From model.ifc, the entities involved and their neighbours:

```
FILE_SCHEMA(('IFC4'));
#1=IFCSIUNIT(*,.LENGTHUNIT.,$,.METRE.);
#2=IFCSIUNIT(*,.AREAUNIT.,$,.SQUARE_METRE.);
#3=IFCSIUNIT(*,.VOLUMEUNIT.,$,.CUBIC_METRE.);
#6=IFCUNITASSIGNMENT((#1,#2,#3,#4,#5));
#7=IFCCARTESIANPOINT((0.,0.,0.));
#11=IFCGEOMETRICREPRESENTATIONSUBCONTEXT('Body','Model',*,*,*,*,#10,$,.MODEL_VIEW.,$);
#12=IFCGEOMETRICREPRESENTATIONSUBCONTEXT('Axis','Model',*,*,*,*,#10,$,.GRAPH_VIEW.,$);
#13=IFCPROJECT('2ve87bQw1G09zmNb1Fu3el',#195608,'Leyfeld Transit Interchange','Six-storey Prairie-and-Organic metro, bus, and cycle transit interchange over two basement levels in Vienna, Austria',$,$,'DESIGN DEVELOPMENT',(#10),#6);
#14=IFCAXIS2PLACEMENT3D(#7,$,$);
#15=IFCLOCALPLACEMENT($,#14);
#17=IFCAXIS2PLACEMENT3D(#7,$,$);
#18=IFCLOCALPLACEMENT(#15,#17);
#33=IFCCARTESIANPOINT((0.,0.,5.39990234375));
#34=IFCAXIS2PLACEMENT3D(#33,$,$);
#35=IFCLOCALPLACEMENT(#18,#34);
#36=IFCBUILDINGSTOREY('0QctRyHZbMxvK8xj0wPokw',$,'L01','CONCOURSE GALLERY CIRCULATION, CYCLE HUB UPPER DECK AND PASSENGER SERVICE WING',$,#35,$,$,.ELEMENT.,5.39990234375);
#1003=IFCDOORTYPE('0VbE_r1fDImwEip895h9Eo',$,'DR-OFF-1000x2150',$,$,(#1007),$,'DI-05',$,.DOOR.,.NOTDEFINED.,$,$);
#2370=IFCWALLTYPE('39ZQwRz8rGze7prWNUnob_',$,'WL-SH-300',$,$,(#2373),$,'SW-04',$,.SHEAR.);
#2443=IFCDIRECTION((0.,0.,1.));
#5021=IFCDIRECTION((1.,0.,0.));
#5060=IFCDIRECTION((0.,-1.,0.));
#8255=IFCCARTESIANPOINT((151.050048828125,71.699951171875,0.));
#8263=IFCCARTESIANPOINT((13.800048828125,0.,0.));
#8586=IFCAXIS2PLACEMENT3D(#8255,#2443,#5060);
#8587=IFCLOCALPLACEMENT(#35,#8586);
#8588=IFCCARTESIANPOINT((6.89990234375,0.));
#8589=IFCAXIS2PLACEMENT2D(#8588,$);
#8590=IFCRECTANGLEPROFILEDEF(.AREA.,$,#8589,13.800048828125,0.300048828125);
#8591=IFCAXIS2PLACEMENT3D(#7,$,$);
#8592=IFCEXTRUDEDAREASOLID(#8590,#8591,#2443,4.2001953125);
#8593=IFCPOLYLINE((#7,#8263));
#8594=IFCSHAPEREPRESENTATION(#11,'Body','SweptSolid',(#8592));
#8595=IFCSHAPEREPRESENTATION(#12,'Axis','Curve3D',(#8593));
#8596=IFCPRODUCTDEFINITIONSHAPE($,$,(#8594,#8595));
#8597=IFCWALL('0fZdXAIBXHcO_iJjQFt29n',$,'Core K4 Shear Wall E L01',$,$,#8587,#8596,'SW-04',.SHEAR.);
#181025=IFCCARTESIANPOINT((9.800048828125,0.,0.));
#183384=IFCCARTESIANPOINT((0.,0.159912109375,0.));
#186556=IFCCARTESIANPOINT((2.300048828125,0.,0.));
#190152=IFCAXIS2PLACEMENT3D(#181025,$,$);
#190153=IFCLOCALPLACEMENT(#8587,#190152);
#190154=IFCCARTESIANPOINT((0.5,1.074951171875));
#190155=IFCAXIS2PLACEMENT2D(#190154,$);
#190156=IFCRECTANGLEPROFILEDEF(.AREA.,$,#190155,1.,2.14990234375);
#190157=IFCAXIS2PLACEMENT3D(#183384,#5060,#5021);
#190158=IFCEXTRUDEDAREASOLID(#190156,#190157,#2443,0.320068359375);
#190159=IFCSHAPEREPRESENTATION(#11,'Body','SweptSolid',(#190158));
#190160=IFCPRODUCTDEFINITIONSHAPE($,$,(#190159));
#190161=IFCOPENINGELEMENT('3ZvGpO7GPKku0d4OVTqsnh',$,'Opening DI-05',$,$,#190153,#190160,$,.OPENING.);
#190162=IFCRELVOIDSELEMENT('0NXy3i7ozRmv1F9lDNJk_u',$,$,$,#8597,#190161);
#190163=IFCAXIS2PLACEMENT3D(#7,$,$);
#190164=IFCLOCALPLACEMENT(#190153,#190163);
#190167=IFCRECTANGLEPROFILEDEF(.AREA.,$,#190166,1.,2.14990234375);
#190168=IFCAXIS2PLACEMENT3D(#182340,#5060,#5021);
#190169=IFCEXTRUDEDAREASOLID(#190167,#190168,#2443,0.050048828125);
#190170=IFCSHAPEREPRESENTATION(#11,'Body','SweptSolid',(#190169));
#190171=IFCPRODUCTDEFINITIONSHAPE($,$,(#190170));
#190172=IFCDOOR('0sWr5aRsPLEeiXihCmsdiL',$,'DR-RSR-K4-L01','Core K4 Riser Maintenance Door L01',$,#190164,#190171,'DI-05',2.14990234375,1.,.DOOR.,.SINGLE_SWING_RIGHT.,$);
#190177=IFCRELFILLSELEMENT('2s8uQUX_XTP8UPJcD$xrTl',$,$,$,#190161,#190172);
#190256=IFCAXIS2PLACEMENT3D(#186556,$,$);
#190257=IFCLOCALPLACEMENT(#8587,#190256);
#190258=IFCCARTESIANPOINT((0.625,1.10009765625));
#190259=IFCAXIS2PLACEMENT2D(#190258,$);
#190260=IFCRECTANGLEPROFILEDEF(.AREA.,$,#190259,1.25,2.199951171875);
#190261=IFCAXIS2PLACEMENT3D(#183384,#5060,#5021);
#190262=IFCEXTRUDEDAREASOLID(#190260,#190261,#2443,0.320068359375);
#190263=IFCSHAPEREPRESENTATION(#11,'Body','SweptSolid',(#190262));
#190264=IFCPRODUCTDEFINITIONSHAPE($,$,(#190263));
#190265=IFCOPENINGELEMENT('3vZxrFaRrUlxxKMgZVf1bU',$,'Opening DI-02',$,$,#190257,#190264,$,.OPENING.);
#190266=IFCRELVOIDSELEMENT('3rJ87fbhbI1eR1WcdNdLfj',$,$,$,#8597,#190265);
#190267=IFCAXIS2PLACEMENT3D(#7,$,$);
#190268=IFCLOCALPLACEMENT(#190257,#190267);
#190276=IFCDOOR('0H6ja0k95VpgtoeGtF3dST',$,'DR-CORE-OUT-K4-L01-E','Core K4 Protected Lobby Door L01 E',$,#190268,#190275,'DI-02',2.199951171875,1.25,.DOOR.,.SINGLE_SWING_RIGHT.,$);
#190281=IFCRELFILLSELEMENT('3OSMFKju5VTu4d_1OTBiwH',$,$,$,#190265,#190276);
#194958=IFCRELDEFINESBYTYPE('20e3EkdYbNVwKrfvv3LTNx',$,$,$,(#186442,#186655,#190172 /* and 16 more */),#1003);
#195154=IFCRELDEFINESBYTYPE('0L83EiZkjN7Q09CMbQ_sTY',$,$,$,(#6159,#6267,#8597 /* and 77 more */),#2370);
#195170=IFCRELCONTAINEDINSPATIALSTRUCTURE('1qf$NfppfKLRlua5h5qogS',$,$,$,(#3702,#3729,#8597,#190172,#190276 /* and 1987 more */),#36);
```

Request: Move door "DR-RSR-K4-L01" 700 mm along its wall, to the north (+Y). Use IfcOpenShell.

```python
import ifcopenshell
import ifcopenshell.api.geometry
import ifcopenshell.util.placement

model = ifcopenshell.open("model.ifc")

door = model.by_id(190172)
opening = door.FillsVoids[0].RelatingOpeningElement
wall = opening.VoidsElements[0].RelatingBuildingElement

wall_matrix = ifcopenshell.util.placement.get_local_placement(wall.ObjectPlacement)
shift = wall_matrix[:3, 0] * -0.7
before = ifcopenshell.util.placement.get_local_placement(door.ObjectPlacement)[:3, 3].copy()

# The door is placed relative to its opening, so it follows when the opening moves.
matrix = ifcopenshell.util.placement.get_local_placement(opening.ObjectPlacement)
matrix[:3, 3] += shift
ifcopenshell.api.geometry.edit_object_placement(
    model, product=opening, matrix=matrix, is_si=False, should_transform_children=True
)

after = ifcopenshell.util.placement.get_local_placement(door.ObjectPlacement)[:3, 3]
print("door moved by", (after - before).round(3) + 0.0)

model.write("model_v2.ifc")
```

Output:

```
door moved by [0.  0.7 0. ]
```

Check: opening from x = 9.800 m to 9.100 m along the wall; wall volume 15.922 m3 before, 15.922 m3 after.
